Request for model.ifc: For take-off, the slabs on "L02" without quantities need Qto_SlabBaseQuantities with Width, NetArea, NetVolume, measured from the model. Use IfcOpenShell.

First a look at what the model holds.

```python
import ifcopenshell
import ifcopenshell.util.element
import ifcopenshell.util.unit

model = ifcopenshell.open("model.ifc")
print(model.schema)
for unit_type in ("LENGTHUNIT", "AREAUNIT", "VOLUMEUNIT"):
    print(unit_type, ifcopenshell.util.unit.calculate_unit_scale(model, unit_type))
storey = next(s for s in model.by_type("IfcBuildingStorey") if s.Name == "L02")
slabs = [e for e in ifcopenshell.util.element.get_decomposition(storey) if e.is_a("IfcSlab")]
for e in sorted(slabs, key=lambda e: e.id()):
    print(e.id(), e.is_a(), e.Name, list(ifcopenshell.util.element.get_psets(e, qtos_only=True)), sep=" | ")
```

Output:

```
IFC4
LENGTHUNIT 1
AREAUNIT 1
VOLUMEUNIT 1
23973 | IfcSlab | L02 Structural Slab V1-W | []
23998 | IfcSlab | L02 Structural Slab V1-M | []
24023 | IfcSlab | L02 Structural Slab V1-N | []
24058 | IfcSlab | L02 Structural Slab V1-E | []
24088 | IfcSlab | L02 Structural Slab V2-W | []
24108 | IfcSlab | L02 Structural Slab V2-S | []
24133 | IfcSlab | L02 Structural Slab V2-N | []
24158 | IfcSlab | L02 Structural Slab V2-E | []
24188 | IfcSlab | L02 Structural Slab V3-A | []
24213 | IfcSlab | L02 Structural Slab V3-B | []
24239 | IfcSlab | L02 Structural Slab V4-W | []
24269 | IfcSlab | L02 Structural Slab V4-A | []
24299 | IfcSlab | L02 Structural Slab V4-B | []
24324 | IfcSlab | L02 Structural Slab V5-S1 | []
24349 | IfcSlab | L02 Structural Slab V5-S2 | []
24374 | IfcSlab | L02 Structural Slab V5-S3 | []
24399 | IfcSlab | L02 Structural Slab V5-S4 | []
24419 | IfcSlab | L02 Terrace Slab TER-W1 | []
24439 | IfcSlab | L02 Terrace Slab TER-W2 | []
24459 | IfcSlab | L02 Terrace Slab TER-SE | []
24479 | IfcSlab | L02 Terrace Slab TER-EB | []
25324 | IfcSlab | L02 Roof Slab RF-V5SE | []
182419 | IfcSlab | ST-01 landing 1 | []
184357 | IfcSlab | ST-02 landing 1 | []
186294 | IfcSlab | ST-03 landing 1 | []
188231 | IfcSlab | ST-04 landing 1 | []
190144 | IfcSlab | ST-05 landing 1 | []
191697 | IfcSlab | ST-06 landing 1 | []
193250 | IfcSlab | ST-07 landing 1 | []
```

```python
import ifcopenshell
import ifcopenshell.api.pset
import ifcopenshell.geom
import ifcopenshell.util.element
import ifcopenshell.util.shape
import ifcopenshell.util.unit

model = ifcopenshell.open("model.ifc")
unit_scale = ifcopenshell.util.unit.calculate_unit_scale(model)
area_scale = ifcopenshell.util.unit.calculate_unit_scale(model, "AREAUNIT")
volume_scale = ifcopenshell.util.unit.calculate_unit_scale(model, "VOLUMEUNIT")
settings = ifcopenshell.geom.settings()

storey = next(s for s in model.by_type("IfcBuildingStorey") if s.Name == "L02")
slabs = [e for e in ifcopenshell.util.element.get_decomposition(storey) if e.is_a("IfcSlab")]

for e in sorted(slabs, key=lambda e: e.id()):
    if ifcopenshell.util.element.get_psets(e, qtos_only=True, should_inherit=False):
        continue
    # Geometry comes back in metres, in the element's own axes.
    shape = ifcopenshell.geom.create_shape(settings, e)
    values = {
        "Width": ifcopenshell.util.shape.get_z(shape.geometry) / unit_scale,
        "NetArea": ifcopenshell.util.shape.get_footprint_area(shape.geometry) / area_scale,
        "NetVolume": ifcopenshell.util.shape.get_volume(shape.geometry) / volume_scale,
    }
    qto = ifcopenshell.api.pset.add_qto(model, product=e, name="Qto_SlabBaseQuantities")
    ifcopenshell.api.pset.edit_qto(model, qto=qto, properties=values)
    print(e.id(), {k: round(v, 3) for k, v in values.items()})

model.write("model_edited.ifc")
```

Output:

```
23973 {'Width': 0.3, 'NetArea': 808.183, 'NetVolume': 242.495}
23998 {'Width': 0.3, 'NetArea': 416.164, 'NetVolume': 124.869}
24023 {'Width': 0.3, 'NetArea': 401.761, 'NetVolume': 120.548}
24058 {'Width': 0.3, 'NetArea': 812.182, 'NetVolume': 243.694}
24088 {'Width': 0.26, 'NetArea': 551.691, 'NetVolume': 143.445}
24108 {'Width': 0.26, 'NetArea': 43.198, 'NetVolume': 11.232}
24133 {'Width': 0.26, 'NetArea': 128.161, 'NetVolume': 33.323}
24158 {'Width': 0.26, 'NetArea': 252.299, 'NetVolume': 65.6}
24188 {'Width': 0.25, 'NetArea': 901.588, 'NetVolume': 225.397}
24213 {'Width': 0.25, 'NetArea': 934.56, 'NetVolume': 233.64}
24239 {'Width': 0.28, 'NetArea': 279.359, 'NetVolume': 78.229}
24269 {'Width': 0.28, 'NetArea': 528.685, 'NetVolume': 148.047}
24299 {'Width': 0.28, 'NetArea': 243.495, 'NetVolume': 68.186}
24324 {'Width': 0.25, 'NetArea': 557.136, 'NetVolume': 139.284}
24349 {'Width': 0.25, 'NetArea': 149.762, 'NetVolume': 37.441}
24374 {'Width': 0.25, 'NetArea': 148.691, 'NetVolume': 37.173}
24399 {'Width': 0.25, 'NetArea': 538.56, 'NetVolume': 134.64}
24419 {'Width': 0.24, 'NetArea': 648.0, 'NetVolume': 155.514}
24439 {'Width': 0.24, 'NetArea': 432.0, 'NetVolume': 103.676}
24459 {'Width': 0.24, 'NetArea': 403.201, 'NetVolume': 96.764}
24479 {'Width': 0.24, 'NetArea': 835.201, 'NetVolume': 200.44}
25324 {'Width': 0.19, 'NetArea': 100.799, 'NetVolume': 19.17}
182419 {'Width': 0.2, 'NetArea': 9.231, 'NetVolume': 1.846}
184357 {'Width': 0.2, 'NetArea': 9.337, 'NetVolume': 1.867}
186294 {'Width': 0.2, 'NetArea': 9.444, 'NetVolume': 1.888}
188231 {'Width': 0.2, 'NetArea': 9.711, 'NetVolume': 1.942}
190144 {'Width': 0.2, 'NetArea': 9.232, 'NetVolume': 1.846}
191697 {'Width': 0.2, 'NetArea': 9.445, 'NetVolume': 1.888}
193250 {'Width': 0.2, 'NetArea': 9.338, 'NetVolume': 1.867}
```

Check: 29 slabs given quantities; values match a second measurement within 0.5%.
